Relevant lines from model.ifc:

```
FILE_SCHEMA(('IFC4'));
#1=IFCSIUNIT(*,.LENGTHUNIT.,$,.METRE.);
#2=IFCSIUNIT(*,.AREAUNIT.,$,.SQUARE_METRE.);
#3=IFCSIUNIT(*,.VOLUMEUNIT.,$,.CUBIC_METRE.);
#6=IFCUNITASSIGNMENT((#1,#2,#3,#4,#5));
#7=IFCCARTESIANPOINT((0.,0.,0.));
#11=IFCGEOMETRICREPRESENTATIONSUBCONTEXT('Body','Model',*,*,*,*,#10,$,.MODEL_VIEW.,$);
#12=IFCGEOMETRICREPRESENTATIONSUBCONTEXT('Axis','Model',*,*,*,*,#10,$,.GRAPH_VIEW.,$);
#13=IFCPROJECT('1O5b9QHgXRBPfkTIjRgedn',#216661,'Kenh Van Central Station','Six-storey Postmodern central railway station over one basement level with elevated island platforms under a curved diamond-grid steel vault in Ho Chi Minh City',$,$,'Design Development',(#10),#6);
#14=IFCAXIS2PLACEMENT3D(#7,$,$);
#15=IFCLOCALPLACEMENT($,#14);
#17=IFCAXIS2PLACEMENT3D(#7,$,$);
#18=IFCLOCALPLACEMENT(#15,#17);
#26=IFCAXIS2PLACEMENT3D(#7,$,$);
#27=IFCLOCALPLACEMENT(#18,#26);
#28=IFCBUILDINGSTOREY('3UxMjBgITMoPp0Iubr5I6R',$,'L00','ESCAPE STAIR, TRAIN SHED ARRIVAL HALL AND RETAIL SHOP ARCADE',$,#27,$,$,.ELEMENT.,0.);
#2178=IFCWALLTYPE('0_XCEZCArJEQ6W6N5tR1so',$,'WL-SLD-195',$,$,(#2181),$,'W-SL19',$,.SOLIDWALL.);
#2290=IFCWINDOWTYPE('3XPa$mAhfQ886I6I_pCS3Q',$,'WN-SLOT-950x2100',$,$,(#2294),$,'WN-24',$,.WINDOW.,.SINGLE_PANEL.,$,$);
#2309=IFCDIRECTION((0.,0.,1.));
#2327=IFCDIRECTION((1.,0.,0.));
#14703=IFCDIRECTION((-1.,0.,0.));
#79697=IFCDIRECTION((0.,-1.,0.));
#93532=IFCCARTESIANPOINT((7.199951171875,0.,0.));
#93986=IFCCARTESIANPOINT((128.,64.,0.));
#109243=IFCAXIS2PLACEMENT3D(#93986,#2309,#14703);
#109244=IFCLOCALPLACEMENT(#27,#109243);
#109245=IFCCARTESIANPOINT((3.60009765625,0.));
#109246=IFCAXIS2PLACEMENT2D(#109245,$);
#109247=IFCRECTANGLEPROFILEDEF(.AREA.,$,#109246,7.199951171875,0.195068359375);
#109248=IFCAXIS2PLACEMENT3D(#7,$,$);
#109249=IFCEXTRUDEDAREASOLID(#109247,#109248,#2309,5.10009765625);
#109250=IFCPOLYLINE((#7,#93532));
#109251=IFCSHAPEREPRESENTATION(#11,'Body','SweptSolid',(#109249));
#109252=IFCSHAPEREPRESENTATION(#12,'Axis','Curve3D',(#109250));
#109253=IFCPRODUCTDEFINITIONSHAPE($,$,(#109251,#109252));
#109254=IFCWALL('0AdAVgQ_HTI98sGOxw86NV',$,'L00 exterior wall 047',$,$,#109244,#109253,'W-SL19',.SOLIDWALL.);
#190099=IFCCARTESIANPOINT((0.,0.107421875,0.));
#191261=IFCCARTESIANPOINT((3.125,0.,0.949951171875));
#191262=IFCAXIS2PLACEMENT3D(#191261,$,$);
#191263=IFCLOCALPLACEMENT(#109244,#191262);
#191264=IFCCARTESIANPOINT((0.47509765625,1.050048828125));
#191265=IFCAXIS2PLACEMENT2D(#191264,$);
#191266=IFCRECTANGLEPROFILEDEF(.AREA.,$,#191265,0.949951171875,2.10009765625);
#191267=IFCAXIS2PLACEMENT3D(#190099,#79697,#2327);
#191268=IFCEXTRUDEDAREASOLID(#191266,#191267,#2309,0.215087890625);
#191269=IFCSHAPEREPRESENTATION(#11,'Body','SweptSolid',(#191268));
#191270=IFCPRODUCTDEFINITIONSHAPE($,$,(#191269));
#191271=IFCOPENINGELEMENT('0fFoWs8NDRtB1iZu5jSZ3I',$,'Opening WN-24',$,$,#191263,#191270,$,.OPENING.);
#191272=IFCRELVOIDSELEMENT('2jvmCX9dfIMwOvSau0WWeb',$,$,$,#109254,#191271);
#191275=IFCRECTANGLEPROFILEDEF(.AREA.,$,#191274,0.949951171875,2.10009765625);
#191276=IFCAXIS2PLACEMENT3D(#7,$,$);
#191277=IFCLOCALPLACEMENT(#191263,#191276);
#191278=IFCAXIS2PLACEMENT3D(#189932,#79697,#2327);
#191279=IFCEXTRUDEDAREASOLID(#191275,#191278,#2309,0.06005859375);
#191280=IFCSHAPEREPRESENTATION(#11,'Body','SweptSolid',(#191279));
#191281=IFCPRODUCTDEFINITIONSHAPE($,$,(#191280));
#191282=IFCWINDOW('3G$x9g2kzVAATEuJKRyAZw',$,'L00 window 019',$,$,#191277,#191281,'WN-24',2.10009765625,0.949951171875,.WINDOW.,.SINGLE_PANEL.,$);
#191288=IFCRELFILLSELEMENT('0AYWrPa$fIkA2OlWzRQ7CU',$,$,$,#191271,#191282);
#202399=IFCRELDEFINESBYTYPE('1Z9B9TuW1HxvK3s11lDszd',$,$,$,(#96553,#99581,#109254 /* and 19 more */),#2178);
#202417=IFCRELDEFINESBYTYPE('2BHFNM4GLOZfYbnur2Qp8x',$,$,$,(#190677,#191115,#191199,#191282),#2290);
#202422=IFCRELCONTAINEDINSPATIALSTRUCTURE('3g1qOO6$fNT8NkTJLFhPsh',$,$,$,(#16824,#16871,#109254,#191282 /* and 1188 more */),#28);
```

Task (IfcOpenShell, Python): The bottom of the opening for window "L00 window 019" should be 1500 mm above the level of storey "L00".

```python
import numpy as np
import ifcopenshell
import ifcopenshell.api.geometry
import ifcopenshell.geom
import ifcopenshell.util.element
import ifcopenshell.util.placement
import ifcopenshell.util.shape
import ifcopenshell.util.unit

model = ifcopenshell.open("model.ifc")
unit_scale = ifcopenshell.util.unit.calculate_unit_scale(model)

window = model.by_guid("3G$x9g2kzVAATEuJKRyAZw")
opening = window.FillsVoids[0].RelatingOpeningElement
storey = ifcopenshell.util.element.get_container(window, ifc_class="IfcBuildingStorey")
level = ifcopenshell.util.placement.get_local_placement(storey.ObjectPlacement)[2, 3]

# The opening's origin need not be at the sill, so measure its lowest point.
shape = ifcopenshell.geom.create_shape(ifcopenshell.geom.settings(), opening)
bottom = ifcopenshell.util.shape.get_shape_bottom_elevation(shape, shape.geometry) / unit_scale
dz = level + 1.5 - bottom

shift = np.array([0.0, 0.0, dz])
# The window is placed relative to its opening, so it follows when the opening moves.
matrix = ifcopenshell.util.placement.get_local_placement(opening.ObjectPlacement)
matrix[:3, 3] += shift
ifcopenshell.api.geometry.edit_object_placement(
    model, product=opening, matrix=matrix, is_si=False, should_transform_children=True
)

print(f"moved by {dz * unit_scale:+.3f} m")

model.write("model-out.ifc")
```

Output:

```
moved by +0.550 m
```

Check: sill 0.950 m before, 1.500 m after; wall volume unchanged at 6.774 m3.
